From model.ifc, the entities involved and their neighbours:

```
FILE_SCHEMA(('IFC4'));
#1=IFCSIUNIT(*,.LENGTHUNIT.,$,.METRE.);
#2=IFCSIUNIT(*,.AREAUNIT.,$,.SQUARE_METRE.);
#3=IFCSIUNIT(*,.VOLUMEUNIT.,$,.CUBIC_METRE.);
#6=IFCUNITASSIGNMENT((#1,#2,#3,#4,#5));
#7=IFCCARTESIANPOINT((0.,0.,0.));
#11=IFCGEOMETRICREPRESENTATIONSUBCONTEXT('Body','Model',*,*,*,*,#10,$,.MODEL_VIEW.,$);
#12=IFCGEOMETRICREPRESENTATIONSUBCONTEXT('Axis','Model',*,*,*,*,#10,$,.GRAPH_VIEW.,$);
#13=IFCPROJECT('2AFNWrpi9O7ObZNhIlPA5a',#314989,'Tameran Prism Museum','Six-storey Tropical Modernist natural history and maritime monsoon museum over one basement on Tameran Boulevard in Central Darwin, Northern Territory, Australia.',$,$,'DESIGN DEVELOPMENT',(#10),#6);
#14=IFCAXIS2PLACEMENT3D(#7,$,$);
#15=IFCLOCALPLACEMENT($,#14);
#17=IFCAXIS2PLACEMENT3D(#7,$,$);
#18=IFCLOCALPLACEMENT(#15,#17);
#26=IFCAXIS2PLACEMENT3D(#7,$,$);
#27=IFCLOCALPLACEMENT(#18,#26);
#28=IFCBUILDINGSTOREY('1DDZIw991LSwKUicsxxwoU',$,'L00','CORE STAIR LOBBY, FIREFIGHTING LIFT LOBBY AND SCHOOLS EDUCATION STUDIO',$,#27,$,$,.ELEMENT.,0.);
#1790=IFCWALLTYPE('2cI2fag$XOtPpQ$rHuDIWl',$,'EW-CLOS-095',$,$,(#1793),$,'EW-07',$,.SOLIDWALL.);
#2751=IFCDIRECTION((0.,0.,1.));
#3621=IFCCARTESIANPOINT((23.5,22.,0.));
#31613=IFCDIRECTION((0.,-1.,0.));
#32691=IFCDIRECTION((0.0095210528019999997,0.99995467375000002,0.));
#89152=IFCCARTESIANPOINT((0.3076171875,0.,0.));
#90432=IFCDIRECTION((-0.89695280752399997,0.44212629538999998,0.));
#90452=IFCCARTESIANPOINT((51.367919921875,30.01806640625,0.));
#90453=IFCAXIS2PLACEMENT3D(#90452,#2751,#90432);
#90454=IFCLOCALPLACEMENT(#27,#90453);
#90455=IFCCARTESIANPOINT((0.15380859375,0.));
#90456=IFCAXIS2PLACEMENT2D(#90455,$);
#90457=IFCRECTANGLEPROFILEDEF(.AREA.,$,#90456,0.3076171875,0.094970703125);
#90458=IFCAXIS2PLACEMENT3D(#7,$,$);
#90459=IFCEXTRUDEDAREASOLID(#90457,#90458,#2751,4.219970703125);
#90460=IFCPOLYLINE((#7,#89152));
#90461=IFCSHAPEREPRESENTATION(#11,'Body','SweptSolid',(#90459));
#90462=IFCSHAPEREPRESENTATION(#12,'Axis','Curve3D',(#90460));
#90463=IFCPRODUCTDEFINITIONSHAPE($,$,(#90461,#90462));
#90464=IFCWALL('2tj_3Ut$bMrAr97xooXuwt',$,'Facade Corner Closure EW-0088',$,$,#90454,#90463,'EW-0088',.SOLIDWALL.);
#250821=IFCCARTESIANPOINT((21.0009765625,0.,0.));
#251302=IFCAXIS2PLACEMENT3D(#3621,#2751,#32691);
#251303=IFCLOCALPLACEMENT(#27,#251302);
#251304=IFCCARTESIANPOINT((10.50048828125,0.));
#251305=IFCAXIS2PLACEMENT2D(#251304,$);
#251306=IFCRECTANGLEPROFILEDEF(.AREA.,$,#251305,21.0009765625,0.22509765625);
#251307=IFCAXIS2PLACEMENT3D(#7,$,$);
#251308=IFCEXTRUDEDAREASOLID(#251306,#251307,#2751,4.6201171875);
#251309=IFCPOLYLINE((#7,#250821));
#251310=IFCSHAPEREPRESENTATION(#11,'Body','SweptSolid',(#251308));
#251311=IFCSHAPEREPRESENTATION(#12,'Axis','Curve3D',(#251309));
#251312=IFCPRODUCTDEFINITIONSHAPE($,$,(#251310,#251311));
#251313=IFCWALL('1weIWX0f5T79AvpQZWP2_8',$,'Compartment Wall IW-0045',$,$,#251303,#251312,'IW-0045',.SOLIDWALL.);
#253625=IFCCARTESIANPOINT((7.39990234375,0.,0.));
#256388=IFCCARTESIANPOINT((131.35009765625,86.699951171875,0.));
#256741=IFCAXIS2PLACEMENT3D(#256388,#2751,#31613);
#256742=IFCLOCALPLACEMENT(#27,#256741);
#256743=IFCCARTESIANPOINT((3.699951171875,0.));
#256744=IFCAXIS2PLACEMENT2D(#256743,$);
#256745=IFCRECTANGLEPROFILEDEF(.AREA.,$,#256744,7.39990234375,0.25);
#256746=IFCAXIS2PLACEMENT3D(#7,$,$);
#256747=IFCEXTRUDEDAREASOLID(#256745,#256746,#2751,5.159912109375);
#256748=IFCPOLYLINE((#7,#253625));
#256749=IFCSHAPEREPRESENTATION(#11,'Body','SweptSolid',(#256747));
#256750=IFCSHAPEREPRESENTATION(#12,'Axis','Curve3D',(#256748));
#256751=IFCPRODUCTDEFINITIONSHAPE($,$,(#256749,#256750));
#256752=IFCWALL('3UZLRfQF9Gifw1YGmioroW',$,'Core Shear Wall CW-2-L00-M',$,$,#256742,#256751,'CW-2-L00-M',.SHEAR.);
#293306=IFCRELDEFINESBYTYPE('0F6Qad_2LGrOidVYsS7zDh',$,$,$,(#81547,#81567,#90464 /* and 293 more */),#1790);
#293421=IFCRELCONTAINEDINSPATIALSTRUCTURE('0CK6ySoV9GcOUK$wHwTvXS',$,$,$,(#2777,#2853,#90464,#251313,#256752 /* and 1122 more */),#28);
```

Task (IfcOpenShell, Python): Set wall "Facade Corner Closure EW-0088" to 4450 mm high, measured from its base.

```python
import ifcopenshell
import ifcopenshell.geom
import ifcopenshell.util.representation
import ifcopenshell.util.shape

model = ifcopenshell.open("model.ifc")
settings = ifcopenshell.geom.settings()


def volume(element):
    """Net volume in cubic metres, openings subtracted."""
    shape = ifcopenshell.geom.create_shape(settings, element)
    return ifcopenshell.util.shape.get_volume(shape.geometry)


wall = model.by_id(90464)
before = volume(wall)

body = ifcopenshell.util.representation.get_representation(wall, "Model", "Body")
solid = body.Items[0]
old_height = solid.Depth
solid.Depth = 4.45
after = volume(wall)

print(f"height {old_height:g} -> {solid.Depth:g}, volume {before:.3f} -> {after:.3f} m3")

model.write("model_updated.ifc")
```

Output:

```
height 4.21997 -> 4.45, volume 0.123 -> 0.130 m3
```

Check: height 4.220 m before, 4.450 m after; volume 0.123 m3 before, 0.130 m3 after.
